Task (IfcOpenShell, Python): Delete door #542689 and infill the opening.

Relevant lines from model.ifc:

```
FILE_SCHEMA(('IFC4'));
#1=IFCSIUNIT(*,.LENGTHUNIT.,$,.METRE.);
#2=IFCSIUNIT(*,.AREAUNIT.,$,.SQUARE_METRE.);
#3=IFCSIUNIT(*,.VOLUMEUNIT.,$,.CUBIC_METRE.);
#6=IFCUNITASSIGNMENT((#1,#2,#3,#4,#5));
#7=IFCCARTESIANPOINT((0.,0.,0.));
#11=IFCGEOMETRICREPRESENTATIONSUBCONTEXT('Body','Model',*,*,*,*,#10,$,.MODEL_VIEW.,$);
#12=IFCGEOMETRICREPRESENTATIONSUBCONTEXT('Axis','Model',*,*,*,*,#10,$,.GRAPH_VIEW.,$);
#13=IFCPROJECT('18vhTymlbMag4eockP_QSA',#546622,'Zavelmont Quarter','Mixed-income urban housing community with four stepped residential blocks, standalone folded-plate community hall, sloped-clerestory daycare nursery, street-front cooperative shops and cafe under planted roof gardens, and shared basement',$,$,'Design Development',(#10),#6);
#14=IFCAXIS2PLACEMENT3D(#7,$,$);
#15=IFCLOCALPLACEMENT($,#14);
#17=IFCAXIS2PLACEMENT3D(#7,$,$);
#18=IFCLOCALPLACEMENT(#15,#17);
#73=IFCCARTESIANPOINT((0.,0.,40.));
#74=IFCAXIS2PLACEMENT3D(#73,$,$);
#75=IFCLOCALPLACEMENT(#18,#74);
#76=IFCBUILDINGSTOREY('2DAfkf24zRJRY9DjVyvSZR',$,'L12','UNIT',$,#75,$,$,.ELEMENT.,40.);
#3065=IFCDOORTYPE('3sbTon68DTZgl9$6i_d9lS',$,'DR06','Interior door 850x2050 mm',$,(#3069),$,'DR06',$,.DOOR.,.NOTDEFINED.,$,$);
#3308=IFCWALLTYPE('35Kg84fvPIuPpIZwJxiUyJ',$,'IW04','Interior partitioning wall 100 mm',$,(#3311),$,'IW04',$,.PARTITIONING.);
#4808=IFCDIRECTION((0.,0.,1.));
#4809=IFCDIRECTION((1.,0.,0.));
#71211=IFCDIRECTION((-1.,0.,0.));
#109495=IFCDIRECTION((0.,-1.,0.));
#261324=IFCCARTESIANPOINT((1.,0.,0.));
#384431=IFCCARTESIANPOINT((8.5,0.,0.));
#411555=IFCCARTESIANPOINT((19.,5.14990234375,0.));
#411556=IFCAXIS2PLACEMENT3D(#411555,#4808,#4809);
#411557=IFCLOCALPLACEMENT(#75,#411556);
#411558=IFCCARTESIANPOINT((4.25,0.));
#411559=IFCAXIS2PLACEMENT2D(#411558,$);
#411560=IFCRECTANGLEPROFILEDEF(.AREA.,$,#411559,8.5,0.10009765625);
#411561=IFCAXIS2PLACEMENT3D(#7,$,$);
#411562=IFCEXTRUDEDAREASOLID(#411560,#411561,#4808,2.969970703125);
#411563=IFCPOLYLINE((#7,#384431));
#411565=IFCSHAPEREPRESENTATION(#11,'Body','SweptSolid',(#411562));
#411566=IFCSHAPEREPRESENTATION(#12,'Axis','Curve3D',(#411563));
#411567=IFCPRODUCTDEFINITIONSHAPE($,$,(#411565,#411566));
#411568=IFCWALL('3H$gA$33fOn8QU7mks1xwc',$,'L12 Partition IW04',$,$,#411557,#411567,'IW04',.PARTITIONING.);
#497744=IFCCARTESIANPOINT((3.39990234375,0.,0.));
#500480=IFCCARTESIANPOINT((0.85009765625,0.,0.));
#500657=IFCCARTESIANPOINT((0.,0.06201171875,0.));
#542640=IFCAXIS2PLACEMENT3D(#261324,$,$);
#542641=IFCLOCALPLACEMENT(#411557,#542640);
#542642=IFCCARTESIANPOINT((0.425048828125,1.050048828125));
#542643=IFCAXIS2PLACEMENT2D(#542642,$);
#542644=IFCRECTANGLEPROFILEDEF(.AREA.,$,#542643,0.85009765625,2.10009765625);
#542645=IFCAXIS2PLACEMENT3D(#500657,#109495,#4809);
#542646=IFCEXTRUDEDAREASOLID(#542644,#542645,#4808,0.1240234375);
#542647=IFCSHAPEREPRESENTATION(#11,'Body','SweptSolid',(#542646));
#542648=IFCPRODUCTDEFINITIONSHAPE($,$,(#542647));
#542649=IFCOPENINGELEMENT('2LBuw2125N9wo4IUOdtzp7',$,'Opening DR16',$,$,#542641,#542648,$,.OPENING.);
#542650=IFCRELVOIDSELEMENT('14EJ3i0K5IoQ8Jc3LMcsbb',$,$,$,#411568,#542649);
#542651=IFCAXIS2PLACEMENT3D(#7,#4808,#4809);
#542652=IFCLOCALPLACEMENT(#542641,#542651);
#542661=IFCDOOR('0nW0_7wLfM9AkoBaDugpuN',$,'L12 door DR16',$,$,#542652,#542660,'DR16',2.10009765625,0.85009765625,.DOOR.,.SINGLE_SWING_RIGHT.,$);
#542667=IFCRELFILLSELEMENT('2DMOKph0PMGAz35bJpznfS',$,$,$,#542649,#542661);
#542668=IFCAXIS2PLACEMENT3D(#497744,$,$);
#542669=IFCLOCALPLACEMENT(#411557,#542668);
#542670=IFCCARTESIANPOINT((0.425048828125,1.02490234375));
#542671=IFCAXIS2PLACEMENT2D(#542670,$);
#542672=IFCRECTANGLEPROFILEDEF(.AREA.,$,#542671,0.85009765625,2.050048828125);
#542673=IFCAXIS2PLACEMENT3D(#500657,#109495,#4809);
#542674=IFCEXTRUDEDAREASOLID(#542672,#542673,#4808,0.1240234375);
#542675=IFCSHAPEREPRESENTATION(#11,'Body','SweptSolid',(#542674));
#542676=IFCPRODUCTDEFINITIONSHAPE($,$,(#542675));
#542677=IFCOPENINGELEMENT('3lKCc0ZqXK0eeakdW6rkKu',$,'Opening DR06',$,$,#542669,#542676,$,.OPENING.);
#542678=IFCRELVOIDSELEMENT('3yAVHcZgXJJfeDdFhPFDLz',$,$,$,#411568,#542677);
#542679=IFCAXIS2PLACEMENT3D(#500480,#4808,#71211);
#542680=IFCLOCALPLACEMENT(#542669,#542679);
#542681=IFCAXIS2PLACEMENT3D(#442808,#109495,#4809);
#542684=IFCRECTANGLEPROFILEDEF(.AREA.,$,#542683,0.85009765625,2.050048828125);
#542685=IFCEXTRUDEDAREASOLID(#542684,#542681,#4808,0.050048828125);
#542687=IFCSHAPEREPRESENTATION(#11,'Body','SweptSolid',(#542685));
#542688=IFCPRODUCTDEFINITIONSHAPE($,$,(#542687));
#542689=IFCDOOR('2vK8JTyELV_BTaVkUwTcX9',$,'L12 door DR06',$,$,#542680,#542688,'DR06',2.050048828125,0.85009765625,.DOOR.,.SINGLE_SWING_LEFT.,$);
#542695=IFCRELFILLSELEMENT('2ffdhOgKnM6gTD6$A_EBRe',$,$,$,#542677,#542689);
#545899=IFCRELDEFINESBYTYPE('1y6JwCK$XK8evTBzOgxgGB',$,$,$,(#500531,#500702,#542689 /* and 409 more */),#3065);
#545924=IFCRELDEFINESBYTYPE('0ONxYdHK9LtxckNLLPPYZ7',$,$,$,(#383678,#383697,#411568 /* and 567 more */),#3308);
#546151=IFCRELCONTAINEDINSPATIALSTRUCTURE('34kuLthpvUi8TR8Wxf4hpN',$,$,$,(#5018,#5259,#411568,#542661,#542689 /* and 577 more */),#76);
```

```python
import ifcopenshell
import ifcopenshell.api.feature
import ifcopenshell.api.root
import ifcopenshell.geom
import ifcopenshell.util.shape

model = ifcopenshell.open("model.ifc")
settings = ifcopenshell.geom.settings()


def volume(element):
    """Net volume in cubic metres, openings subtracted."""
    shape = ifcopenshell.geom.create_shape(settings, element)
    return ifcopenshell.util.shape.get_volume(shape.geometry)


door = model.by_guid("2vK8JTyELV_BTaVkUwTcX9")
opening = door.FillsVoids[0].RelatingOpeningElement
wall = opening.VoidsElements[0].RelatingBuildingElement
before = volume(wall)

ifcopenshell.api.root.remove_product(model, product=door)
ifcopenshell.api.feature.remove_feature(model, feature=opening)

after = volume(wall)

print(f"wall volume {before:.3f} -> {after:.3f} m3")

model.write("model_updated.ifc")
```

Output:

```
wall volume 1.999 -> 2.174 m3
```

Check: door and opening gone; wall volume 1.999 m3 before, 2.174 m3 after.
